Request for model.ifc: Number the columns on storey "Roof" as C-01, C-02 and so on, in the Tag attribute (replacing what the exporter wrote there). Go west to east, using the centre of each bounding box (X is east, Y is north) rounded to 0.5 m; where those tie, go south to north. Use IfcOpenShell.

First a look at what the model holds.

```python
import ifcopenshell
import ifcopenshell.util.element
import ifcopenshell.util.placement

model = ifcopenshell.open("model.ifc")
print(model.schema)
storey = next(s for s in model.by_type("IfcBuildingStorey") if s.Name == "Roof")
columns = [e for e in ifcopenshell.util.element.get_decomposition(storey) if e.is_a("IfcColumn")]
for e in sorted(columns, key=lambda e: e.id()):
    origin = ifcopenshell.util.placement.get_local_placement(e.ObjectPlacement)[:3, 3]
    print(e.id(), e.Tag, e.Name, origin.round(2) + 0.0, sep=" | ")
```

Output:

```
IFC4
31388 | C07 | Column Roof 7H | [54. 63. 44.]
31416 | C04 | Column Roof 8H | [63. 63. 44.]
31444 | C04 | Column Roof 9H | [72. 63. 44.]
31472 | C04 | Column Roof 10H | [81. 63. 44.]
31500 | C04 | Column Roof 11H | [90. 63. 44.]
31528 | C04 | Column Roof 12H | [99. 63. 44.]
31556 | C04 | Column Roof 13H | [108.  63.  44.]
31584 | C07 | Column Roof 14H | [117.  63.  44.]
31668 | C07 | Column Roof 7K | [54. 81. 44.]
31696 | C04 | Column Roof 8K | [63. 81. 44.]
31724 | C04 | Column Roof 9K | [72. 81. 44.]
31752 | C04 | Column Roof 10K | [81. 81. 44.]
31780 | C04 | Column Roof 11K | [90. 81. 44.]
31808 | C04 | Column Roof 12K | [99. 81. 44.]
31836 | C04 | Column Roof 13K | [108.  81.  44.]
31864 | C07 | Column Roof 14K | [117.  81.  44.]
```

```python
import ifcopenshell
import ifcopenshell.geom
import ifcopenshell.util.element
import ifcopenshell.util.shape

model = ifcopenshell.open("model.ifc")
settings = ifcopenshell.geom.settings()
settings.set("use-world-coords", True)


def centre(element):
    shape = ifcopenshell.geom.create_shape(settings, element)
    return ifcopenshell.util.shape.get_bbox_centroid(shape.geometry)


storey = next(s for s in model.by_type("IfcBuildingStorey") if s.Name == "Roof")
columns = [e for e in ifcopenshell.util.element.get_decomposition(storey) if e.is_a("IfcColumn")]

# Insertion points can sit at a corner or the storey origin, so sort by the geometry (in metres).
centres = {e: centre(e) for e in columns}
columns.sort(key=lambda e: (round(centres[e][0] / 0.5), centres[e][1]))

for i, e in enumerate(columns, start=1):
    number = f"C-{i:02d}"
    e.Tag = number
    print(e.id(), number)

model.write("model_v2.ifc")
```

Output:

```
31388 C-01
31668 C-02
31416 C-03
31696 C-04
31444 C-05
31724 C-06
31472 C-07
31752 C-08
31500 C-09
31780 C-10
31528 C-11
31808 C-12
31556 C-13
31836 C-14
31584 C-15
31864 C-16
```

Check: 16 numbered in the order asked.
